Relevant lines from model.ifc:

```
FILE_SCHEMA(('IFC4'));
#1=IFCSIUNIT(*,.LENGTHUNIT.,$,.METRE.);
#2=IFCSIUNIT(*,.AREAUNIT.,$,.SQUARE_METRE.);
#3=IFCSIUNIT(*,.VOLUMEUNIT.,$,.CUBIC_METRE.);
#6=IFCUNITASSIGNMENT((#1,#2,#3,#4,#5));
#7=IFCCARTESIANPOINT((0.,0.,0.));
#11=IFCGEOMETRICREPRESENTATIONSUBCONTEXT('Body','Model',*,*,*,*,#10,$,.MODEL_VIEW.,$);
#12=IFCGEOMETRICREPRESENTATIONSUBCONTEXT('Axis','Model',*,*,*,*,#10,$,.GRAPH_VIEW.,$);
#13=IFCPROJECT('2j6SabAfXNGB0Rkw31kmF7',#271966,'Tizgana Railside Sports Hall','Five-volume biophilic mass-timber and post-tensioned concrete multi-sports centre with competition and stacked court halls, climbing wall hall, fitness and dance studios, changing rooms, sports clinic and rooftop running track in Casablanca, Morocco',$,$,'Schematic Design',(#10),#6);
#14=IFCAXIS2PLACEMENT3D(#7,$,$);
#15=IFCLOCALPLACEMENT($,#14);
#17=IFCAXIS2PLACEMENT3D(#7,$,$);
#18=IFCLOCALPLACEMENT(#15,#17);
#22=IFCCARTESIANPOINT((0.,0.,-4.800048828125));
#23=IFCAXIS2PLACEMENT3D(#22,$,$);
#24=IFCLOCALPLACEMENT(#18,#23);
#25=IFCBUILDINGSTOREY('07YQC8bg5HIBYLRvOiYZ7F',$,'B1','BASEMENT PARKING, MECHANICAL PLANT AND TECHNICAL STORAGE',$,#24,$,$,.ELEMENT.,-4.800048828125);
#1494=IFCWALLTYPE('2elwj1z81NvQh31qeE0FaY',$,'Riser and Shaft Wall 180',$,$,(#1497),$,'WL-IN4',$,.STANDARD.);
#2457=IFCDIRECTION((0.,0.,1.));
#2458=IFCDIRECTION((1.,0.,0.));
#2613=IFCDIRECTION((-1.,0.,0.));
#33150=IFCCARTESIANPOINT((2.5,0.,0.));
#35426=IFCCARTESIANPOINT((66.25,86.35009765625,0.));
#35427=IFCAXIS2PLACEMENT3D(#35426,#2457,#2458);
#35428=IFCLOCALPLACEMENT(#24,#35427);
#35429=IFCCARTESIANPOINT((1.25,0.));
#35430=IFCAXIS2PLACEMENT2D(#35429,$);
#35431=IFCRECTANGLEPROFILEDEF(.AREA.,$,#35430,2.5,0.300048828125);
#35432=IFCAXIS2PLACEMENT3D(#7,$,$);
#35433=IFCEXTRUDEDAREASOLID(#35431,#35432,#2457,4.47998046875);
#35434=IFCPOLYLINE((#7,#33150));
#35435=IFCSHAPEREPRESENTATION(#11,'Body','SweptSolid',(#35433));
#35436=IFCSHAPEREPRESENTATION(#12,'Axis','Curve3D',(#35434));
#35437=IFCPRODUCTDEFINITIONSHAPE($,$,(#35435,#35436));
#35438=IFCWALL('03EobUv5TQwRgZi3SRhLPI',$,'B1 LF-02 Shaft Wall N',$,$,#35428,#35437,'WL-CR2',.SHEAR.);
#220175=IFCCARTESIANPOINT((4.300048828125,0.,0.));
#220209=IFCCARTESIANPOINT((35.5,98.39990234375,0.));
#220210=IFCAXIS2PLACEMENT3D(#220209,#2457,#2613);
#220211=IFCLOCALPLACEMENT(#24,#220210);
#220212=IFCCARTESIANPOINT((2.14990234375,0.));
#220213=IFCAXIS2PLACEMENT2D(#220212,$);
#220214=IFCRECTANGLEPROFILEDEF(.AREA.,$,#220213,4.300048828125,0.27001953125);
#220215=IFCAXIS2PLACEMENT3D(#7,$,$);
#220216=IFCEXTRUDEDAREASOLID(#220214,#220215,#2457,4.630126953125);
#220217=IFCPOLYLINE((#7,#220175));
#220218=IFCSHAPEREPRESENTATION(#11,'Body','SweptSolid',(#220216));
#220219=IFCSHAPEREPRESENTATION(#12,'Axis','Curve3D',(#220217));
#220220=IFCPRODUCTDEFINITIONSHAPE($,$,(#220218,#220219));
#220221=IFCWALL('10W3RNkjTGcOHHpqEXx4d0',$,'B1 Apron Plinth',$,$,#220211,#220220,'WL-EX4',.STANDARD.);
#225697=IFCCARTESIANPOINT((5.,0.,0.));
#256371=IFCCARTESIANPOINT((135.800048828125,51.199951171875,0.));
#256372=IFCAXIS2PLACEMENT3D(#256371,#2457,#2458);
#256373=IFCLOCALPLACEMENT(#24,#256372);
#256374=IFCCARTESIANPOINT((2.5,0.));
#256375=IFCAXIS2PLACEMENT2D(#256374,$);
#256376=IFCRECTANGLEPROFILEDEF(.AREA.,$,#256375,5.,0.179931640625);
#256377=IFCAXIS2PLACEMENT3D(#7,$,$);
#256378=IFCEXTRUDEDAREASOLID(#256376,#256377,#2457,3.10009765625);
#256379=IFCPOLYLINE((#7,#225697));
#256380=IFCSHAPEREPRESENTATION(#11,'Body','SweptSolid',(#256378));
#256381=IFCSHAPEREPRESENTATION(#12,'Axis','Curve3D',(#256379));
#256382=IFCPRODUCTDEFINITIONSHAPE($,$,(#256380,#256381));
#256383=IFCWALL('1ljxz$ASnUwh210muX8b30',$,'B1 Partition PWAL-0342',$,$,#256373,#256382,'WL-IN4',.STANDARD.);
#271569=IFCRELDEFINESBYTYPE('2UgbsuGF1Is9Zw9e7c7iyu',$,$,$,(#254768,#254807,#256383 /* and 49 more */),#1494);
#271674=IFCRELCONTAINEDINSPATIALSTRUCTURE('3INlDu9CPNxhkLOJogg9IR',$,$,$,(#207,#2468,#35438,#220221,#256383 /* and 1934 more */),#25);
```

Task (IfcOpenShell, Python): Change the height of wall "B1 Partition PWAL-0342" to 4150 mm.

```python
import ifcopenshell
import ifcopenshell.geom
import ifcopenshell.util.representation
import ifcopenshell.util.shape

model = ifcopenshell.open("model.ifc")
settings = ifcopenshell.geom.settings()


def volume(element):
    """Net volume in cubic metres, openings subtracted."""
    shape = ifcopenshell.geom.create_shape(settings, element)
    return ifcopenshell.util.shape.get_volume(shape.geometry)


wall = model.by_guid("1ljxz$ASnUwh210muX8b30")
before = volume(wall)

body = ifcopenshell.util.representation.get_representation(wall, "Model", "Body")
solid = body.Items[0]
old_height = solid.Depth
solid.Depth = 4.15
after = volume(wall)

print(f"height {old_height:g} -> {solid.Depth:g}, volume {before:.3f} -> {after:.3f} m3")

model.write("model_v2.ifc")
```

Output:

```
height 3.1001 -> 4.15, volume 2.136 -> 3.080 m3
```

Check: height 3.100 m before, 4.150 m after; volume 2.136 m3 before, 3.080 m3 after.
